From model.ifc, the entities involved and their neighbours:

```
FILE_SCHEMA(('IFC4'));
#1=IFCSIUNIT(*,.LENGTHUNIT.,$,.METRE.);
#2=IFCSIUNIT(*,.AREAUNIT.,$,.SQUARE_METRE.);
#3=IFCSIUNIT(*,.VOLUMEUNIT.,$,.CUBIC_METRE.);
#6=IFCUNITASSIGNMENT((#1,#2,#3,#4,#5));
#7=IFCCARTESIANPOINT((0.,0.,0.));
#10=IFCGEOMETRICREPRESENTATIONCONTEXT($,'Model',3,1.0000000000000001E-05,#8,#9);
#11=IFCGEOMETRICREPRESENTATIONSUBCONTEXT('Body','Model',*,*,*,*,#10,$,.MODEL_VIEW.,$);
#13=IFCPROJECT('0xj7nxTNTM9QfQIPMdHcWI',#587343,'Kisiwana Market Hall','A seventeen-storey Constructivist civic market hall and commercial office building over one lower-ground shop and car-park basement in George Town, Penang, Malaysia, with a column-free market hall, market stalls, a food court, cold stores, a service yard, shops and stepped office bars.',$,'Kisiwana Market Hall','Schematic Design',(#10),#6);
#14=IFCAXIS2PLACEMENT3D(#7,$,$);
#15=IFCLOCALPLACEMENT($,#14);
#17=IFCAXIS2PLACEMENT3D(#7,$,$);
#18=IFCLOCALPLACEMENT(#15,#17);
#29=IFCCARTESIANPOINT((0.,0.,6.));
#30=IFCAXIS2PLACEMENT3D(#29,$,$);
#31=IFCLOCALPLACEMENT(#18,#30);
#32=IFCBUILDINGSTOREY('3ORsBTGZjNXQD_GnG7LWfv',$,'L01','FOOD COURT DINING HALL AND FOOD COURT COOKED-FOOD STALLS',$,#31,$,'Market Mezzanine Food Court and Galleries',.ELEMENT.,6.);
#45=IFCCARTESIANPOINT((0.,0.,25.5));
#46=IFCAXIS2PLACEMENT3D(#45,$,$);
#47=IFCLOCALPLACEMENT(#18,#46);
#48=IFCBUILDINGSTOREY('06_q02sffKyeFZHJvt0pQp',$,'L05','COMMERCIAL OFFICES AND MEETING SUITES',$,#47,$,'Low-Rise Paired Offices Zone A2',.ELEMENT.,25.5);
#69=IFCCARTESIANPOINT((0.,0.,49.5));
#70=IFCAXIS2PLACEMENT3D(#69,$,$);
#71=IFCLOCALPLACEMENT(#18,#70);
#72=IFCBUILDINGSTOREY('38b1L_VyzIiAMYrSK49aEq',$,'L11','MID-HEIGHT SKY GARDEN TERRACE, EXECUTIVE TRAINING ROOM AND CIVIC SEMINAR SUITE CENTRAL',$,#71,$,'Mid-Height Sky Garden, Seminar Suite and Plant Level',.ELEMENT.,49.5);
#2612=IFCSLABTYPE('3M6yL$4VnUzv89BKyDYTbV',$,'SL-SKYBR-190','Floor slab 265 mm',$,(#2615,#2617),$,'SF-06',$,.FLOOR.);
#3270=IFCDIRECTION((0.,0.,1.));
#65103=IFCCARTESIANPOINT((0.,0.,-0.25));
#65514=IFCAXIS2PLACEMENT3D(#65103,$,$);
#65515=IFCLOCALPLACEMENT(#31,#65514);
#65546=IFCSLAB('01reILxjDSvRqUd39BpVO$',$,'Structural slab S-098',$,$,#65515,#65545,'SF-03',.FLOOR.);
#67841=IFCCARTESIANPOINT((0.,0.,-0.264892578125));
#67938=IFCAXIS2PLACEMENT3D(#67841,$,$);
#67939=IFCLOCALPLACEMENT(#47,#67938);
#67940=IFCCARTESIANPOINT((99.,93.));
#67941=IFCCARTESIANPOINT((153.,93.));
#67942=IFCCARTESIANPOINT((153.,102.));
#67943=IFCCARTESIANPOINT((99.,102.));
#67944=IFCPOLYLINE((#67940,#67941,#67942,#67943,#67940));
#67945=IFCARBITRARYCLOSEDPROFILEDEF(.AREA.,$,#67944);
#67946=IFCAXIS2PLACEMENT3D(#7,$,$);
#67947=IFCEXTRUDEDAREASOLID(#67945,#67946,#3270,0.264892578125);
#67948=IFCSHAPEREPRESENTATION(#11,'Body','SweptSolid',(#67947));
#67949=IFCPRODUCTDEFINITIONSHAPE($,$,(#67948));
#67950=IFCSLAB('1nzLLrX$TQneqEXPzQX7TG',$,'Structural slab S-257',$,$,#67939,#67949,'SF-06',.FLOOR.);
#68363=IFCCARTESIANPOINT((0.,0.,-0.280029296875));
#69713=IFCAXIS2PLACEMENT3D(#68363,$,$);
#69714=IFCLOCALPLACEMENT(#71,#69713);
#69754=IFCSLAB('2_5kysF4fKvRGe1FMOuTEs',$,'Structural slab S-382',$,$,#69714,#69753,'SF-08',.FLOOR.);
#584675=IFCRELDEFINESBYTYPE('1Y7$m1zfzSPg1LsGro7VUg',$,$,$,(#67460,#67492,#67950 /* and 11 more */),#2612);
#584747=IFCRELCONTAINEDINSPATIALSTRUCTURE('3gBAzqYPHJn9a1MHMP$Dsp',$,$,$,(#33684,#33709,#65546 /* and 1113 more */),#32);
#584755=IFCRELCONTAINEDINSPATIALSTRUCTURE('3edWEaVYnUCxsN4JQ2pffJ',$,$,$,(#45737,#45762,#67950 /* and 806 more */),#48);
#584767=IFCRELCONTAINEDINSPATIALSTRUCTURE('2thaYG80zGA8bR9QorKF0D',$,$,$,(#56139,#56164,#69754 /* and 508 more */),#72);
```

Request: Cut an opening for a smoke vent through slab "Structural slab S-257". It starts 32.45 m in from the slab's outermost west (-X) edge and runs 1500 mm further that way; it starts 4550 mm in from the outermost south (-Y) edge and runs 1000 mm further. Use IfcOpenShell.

```python
import numpy as np
import ifcopenshell
import ifcopenshell.api.feature
import ifcopenshell.api.geometry
import ifcopenshell.api.root
import ifcopenshell.geom
import ifcopenshell.util.placement
import ifcopenshell.util.representation
import ifcopenshell.util.shape
import ifcopenshell.util.unit

model = ifcopenshell.open("model.ifc")
unit_scale = ifcopenshell.util.unit.calculate_unit_scale(model)
settings = ifcopenshell.geom.settings()


def volume(element):
    """Net volume in cubic metres, openings subtracted."""
    shape = ifcopenshell.geom.create_shape(settings, element)
    return ifcopenshell.util.shape.get_volume(shape.geometry)


slab = model.by_guid("1nzLLrX$TQneqEXPzQX7TG")
before = volume(slab)

# Extent in the slab's own axes, in metres. The edges named are its -X and -Y sides.
slab_shape = ifcopenshell.geom.create_shape(settings, slab)
vertices = ifcopenshell.util.shape.get_vertices(slab_shape.geometry)
x_min, y_min, bottom = vertices.min(axis=0)
top = vertices[:, 2].max()

opening = ifcopenshell.api.root.create_entity(model, ifc_class="IfcOpeningElement", name="Smoke vent opening", predefined_type="OPENING")
context = ifcopenshell.util.representation.get_context(model, "Model", "Body", "MODEL_VIEW")
width, depth = 1.5, 1
outline = [(0.0, 0.0), (width, 0.0), (width, depth), (0.0, depth), (0.0, 0.0)]
# Overshoot both faces by 50 mm so the cut is clean.
shape = ifcopenshell.api.geometry.add_slab_representation(
    model, context=context, depth=top - bottom + 0.1, polyline=outline
)
ifcopenshell.api.geometry.assign_representation(model, product=opening, representation=shape)

matrix = ifcopenshell.util.placement.get_local_placement(slab.ObjectPlacement)
matrix[:, 3] = matrix @ np.append(np.array([x_min + 32.45, y_min + 4.55, bottom - 0.05]) / unit_scale, 1.0)
ifcopenshell.api.geometry.edit_object_placement(model, product=opening, matrix=matrix, is_si=False)
ifcopenshell.api.feature.add_feature(model, feature=opening, element=slab)

after = volume(slab)

print(f"slab volume {before:.3f} -> {after:.3f} m3")

model.write("model-out.ifc")
```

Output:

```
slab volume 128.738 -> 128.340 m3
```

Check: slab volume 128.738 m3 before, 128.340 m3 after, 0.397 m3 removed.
